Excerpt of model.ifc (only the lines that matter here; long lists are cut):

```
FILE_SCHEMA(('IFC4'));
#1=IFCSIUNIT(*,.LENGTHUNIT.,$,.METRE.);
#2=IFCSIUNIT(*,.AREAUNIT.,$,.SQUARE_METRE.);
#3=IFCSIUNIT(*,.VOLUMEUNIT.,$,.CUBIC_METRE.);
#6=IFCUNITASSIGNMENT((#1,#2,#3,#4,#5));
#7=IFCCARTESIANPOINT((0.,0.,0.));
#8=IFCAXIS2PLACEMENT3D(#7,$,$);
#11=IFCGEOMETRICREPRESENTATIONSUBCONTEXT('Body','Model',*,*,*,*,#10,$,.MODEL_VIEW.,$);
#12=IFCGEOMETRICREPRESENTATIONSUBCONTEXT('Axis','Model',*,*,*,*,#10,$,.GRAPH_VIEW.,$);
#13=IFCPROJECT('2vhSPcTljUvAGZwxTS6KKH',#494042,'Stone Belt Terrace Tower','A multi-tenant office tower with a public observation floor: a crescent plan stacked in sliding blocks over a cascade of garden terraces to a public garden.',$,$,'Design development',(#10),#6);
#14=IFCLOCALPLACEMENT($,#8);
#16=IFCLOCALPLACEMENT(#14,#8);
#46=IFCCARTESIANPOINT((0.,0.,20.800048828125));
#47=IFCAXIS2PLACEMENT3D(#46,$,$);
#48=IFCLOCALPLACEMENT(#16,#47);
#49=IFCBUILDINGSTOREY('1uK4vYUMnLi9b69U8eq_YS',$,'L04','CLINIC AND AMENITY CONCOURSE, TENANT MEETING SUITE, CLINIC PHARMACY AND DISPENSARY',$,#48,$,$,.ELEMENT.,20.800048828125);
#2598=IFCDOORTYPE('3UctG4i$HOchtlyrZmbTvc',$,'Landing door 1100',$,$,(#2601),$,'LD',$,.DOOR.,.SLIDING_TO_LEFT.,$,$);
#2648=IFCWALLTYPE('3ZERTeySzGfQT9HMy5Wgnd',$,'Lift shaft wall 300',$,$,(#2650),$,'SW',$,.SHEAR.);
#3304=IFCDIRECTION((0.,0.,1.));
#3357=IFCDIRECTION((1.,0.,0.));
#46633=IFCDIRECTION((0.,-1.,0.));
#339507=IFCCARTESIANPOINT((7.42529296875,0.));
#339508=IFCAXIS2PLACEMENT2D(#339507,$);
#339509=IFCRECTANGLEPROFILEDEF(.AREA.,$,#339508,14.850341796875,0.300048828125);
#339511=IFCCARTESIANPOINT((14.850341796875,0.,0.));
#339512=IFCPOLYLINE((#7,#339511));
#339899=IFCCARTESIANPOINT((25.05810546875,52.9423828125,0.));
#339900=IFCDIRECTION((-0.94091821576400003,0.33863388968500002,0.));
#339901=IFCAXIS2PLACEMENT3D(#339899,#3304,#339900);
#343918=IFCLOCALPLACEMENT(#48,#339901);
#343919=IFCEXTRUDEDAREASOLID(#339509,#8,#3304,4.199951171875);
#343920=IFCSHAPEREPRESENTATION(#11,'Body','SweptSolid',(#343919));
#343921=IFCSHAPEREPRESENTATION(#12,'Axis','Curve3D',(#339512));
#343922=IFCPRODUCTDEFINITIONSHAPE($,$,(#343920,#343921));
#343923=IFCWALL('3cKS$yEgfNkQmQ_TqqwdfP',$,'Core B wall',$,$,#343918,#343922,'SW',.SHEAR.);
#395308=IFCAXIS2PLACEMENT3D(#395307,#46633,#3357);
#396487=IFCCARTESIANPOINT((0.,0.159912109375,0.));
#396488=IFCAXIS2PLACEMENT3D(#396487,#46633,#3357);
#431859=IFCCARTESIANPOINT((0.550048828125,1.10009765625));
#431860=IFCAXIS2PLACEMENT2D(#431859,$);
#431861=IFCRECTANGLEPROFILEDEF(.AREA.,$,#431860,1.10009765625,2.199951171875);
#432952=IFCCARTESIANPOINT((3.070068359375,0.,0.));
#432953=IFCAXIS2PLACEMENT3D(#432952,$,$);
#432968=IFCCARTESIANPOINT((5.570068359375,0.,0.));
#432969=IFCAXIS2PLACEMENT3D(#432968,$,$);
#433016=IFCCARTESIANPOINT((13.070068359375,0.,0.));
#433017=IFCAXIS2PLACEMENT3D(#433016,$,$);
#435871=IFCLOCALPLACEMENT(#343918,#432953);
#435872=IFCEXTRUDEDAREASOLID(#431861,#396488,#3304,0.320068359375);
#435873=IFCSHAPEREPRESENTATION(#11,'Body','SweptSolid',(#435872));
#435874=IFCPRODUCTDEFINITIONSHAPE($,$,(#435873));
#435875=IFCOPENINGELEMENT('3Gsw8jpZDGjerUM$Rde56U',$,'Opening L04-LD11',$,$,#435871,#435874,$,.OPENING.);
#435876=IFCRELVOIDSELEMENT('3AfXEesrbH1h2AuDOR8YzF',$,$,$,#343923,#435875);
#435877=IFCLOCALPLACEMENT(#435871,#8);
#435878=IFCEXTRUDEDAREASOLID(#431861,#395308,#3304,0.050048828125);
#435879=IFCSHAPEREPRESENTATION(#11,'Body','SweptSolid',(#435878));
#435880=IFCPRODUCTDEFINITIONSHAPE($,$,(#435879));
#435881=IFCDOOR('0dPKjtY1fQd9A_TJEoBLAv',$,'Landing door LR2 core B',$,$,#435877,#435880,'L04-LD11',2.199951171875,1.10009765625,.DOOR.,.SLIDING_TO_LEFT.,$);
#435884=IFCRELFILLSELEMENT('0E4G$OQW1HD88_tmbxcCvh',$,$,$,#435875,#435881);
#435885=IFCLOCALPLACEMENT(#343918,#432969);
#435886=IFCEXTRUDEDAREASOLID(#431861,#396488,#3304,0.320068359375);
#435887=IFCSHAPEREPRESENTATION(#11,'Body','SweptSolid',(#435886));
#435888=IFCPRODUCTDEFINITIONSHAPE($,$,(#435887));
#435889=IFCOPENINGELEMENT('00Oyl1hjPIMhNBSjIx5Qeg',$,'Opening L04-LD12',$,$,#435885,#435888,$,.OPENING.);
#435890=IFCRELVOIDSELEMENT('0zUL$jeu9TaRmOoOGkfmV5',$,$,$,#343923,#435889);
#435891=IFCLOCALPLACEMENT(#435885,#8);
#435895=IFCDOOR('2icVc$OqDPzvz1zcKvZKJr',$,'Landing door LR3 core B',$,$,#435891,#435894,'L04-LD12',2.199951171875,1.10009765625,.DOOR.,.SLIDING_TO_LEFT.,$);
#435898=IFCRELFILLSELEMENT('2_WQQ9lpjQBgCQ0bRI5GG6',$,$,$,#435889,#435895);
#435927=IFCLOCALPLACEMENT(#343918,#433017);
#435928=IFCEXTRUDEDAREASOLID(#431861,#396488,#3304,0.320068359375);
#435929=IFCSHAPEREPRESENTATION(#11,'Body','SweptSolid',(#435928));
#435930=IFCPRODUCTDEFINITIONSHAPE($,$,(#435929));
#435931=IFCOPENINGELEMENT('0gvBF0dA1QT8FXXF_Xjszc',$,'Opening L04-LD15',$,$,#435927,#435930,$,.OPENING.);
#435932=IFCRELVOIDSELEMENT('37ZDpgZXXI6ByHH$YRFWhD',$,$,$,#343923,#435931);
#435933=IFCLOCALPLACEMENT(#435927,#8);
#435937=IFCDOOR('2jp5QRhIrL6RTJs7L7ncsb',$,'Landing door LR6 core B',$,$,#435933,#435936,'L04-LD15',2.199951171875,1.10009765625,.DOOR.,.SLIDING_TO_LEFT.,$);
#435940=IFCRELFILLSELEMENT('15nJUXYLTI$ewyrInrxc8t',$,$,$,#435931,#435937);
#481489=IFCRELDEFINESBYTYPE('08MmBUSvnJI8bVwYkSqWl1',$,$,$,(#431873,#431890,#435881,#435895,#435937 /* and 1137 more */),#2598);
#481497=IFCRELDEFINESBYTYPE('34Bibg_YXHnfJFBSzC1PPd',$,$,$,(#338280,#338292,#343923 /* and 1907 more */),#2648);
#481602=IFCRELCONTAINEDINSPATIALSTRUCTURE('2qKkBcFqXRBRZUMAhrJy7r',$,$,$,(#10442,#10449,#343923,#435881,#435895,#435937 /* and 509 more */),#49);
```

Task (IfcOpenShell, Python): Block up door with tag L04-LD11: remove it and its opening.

```python
import ifcopenshell
import ifcopenshell.api.feature
import ifcopenshell.api.root
import ifcopenshell.geom
import ifcopenshell.util.shape

model = ifcopenshell.open("model.ifc")
settings = ifcopenshell.geom.settings()


def volume(element):
    """Net volume in cubic metres, openings subtracted."""
    shape = ifcopenshell.geom.create_shape(settings, element)
    return ifcopenshell.util.shape.get_volume(shape.geometry)


door = model.by_guid("0dPKjtY1fQd9A_TJEoBLAv")
opening = door.FillsVoids[0].RelatingOpeningElement
wall = opening.VoidsElements[0].RelatingBuildingElement
before = volume(wall)

ifcopenshell.api.root.remove_product(model, product=door)
ifcopenshell.api.feature.remove_feature(model, feature=opening)

after = volume(wall)

print(f"wall volume {before:.3f} -> {after:.3f} m3")

model.write("model-out.ifc")
```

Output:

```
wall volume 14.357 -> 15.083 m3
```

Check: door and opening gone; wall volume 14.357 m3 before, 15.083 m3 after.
